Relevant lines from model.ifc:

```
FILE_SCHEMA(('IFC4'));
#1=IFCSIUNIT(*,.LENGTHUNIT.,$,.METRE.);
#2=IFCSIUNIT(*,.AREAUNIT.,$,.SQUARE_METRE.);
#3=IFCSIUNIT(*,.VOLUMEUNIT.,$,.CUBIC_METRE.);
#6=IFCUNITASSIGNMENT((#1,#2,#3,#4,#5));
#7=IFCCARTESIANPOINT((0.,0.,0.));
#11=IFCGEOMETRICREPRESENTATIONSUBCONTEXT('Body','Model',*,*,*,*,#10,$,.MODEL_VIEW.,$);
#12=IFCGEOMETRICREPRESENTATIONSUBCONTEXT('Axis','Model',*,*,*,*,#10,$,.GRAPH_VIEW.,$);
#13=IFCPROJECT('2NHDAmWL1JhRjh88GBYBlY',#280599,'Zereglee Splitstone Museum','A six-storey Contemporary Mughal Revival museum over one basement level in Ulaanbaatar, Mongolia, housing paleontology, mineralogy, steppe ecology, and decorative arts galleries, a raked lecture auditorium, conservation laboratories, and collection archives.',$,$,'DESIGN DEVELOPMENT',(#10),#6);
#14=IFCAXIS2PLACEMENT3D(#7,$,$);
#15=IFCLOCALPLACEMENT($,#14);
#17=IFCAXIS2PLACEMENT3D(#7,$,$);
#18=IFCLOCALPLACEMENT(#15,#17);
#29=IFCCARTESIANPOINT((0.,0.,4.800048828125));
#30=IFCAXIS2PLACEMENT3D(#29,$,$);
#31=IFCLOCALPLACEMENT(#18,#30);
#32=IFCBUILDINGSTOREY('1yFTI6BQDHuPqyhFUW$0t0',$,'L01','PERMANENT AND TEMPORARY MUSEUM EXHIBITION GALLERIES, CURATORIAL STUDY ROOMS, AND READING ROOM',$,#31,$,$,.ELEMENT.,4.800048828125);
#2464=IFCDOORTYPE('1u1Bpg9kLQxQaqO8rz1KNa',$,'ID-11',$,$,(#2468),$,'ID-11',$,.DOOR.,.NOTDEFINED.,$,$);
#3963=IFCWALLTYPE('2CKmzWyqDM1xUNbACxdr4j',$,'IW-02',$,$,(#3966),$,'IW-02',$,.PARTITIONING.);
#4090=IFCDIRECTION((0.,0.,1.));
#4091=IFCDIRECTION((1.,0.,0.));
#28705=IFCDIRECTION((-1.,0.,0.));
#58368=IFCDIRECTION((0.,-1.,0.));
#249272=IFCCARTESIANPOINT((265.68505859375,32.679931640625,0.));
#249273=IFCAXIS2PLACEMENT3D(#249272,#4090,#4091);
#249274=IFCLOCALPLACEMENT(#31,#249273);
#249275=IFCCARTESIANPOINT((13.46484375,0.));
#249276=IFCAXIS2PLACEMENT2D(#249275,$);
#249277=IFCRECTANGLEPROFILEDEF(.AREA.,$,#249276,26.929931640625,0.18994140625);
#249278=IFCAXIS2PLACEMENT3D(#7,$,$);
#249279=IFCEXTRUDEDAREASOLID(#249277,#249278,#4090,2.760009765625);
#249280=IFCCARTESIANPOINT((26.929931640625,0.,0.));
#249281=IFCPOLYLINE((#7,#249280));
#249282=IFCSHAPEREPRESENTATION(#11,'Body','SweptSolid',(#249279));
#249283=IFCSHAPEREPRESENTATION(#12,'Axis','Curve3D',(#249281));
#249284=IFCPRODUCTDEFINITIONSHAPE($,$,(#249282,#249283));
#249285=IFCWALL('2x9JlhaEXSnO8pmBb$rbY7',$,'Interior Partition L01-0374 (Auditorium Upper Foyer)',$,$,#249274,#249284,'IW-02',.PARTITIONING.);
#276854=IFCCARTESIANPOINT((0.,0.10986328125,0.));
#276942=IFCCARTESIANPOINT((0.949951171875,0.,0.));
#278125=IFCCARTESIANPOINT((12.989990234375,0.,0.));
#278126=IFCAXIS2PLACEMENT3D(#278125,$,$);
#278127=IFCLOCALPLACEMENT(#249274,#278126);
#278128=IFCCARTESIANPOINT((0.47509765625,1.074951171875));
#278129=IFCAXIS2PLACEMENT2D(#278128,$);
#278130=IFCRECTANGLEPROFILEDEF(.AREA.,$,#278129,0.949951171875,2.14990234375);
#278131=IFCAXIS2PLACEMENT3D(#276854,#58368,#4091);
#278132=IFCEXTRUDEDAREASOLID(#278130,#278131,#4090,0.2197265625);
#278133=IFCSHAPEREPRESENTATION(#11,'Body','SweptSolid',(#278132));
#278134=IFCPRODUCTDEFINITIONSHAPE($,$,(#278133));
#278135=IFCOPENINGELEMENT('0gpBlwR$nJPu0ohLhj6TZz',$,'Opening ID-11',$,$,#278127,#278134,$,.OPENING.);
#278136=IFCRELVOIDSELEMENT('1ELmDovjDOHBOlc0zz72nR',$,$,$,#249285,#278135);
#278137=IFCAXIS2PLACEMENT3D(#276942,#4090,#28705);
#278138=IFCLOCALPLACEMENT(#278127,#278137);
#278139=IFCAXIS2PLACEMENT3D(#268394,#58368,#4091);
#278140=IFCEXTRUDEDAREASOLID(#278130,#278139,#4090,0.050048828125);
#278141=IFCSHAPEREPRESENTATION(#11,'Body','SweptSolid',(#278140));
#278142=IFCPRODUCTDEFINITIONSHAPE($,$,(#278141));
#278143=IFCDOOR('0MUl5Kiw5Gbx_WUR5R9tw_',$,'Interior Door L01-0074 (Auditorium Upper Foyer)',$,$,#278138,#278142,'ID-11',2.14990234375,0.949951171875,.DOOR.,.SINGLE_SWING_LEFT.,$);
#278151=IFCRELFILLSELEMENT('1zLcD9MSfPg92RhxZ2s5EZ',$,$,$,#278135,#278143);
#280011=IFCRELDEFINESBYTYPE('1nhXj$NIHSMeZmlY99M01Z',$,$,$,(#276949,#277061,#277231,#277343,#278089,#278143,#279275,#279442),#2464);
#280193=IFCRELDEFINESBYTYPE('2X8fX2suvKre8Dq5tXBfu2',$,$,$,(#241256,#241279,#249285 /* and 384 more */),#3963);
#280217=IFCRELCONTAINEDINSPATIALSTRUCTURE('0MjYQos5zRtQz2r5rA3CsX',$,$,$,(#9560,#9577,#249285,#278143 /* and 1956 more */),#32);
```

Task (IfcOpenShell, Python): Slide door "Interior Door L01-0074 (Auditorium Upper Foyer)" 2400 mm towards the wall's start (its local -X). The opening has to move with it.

```python
import ifcopenshell
import ifcopenshell.api.geometry
import ifcopenshell.util.placement
import ifcopenshell.util.unit

model = ifcopenshell.open("model.ifc")
unit_scale = ifcopenshell.util.unit.calculate_unit_scale(model)

door = model.by_guid("0MUl5Kiw5Gbx_WUR5R9tw_")
opening = door.FillsVoids[0].RelatingOpeningElement
wall = opening.VoidsElements[0].RelatingBuildingElement

wall_matrix = ifcopenshell.util.placement.get_local_placement(wall.ObjectPlacement)
shift = wall_matrix[:3, 0] * -2.4 / unit_scale
before = ifcopenshell.util.placement.get_local_placement(door.ObjectPlacement)[:3, 3].copy()

# The door is placed relative to its opening, so it follows when the opening moves.
matrix = ifcopenshell.util.placement.get_local_placement(opening.ObjectPlacement)
matrix[:3, 3] += shift
ifcopenshell.api.geometry.edit_object_placement(
    model, product=opening, matrix=matrix, is_si=False, should_transform_children=True
)

after = ifcopenshell.util.placement.get_local_placement(door.ObjectPlacement)[:3, 3]
print("door moved by", (after - before).round(3) + 0.0)

model.write("model-out.ifc")
```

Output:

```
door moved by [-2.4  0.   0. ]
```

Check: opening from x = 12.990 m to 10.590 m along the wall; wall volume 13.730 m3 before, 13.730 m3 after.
